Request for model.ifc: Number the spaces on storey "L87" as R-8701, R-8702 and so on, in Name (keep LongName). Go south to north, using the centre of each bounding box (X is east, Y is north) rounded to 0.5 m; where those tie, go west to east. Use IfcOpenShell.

First a look at what the model holds.

```python
import ifcopenshell
import ifcopenshell.util.element
import ifcopenshell.util.placement

model = ifcopenshell.open("model.ifc")
print(model.schema)
storey = next(s for s in model.by_type("IfcBuildingStorey") if s.Name == "L87")
spaces = [e for e in ifcopenshell.util.element.get_decomposition(storey) if e.is_a("IfcSpace")]
for e in sorted(spaces, key=lambda e: e.id()):
    origin = ifcopenshell.util.placement.get_local_placement(e.ObjectPlacement)[:3, 3]
    print(e.id(), e.Name, e.LongName, origin.round(2) + 0.0, sep=" | ")
```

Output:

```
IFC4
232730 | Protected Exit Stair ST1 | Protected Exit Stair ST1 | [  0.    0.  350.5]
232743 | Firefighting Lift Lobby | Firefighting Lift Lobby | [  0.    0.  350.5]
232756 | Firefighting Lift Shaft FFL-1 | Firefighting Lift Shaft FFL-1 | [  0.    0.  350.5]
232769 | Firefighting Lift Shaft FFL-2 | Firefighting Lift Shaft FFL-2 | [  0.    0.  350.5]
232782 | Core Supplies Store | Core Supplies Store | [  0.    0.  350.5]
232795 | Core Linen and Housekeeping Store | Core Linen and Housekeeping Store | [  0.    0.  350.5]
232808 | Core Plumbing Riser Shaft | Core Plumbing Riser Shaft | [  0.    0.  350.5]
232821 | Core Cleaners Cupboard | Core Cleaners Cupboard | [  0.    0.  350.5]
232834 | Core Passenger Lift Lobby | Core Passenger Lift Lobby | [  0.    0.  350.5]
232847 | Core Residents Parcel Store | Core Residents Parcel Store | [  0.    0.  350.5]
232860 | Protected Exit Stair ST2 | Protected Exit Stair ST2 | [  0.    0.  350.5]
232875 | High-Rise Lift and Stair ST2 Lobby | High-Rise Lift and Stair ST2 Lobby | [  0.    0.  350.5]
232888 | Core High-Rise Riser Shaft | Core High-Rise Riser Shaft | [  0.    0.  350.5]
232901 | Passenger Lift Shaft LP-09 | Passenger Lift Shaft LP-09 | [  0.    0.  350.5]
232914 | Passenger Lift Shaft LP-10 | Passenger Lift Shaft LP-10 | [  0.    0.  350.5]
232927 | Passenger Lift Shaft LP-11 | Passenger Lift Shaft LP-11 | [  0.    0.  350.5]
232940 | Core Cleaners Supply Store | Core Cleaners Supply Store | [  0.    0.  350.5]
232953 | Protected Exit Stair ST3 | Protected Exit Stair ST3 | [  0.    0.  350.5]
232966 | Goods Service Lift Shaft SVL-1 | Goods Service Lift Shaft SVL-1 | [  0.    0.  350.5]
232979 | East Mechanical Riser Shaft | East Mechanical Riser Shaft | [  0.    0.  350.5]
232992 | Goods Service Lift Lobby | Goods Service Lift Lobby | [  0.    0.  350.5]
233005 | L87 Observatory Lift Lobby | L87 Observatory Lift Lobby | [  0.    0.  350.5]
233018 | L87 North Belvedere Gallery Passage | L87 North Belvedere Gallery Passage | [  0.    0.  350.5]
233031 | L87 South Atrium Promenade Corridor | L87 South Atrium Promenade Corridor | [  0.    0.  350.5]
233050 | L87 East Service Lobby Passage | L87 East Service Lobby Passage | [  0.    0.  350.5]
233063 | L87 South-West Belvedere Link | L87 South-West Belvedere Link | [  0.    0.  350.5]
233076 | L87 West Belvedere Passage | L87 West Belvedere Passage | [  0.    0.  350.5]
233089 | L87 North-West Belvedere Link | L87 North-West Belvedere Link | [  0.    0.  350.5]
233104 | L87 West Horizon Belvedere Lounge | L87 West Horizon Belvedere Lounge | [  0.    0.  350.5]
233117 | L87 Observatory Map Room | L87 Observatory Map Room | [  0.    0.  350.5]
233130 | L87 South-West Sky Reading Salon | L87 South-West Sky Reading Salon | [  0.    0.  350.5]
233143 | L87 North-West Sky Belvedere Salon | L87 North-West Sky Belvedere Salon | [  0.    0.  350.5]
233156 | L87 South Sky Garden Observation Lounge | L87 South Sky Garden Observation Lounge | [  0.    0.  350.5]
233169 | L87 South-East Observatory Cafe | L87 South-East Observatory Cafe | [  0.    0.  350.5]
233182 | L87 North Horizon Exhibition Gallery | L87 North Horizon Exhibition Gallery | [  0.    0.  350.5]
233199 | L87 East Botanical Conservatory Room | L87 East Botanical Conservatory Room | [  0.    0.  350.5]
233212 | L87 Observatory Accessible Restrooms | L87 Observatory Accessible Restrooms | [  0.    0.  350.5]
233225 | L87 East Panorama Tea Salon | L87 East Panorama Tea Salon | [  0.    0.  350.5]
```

```python
import ifcopenshell
import ifcopenshell.geom
import ifcopenshell.util.element
import ifcopenshell.util.shape

model = ifcopenshell.open("model.ifc")
settings = ifcopenshell.geom.settings()
settings.set("use-world-coords", True)


def centre(element):
    shape = ifcopenshell.geom.create_shape(settings, element)
    return ifcopenshell.util.shape.get_bbox_centroid(shape.geometry)


storey = next(s for s in model.by_type("IfcBuildingStorey") if s.Name == "L87")
spaces = [e for e in ifcopenshell.util.element.get_decomposition(storey) if e.is_a("IfcSpace")]

# Insertion points can sit at a corner or the storey origin, so sort by the geometry (in metres).
centres = {e: centre(e) for e in spaces}
spaces.sort(key=lambda e: (round(centres[e][1] / 0.5), centres[e][0]))

for i, e in enumerate(spaces, start=1):
    number = f"R-87{i:02d}"
    e.Name = number
    print(e.id(), number)

model.write("model_rev.ifc")
```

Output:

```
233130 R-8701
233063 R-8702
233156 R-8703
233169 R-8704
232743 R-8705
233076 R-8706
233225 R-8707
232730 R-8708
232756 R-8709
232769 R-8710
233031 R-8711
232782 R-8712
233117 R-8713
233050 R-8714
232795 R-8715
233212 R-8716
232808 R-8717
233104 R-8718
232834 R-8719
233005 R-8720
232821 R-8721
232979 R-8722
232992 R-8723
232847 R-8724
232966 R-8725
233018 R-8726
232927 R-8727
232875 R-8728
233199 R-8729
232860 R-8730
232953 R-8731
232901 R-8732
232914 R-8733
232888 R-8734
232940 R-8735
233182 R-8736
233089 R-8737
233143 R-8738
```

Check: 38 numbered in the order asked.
